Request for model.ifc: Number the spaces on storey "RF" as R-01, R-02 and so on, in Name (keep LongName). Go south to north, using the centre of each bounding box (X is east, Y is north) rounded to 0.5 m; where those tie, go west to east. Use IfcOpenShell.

First a look at what the model holds.

```python
import ifcopenshell
import ifcopenshell.util.element
import ifcopenshell.util.placement

model = ifcopenshell.open("model.ifc")
print(model.schema)
storey = next(s for s in model.by_type("IfcBuildingStorey") if s.Name == "RF")
spaces = [e for e in ifcopenshell.util.element.get_decomposition(storey) if e.is_a("IfcSpace")]
for e in sorted(spaces, key=lambda e: e.id()):
    origin = ifcopenshell.util.placement.get_local_placement(e.ObjectPlacement)[:3, 3]
    print(e.id(), e.Name, e.LongName, origin.round(2) + 0.0, sep=" | ")
```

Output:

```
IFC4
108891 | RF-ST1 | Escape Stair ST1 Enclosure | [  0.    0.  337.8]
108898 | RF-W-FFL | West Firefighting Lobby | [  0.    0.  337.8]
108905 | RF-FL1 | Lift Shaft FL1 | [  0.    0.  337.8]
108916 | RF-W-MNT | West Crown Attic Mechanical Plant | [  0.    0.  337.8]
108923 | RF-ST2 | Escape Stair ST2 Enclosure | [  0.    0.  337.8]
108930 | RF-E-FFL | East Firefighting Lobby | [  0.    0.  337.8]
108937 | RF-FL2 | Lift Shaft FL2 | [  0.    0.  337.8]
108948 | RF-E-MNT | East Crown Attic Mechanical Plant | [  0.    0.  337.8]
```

```python
import ifcopenshell
import ifcopenshell.geom
import ifcopenshell.util.element
import ifcopenshell.util.shape

model = ifcopenshell.open("model.ifc")
settings = ifcopenshell.geom.settings()
settings.set("use-world-coords", True)


def centre(element):
    shape = ifcopenshell.geom.create_shape(settings, element)
    return ifcopenshell.util.shape.get_bbox_centroid(shape.geometry)


storey = next(s for s in model.by_type("IfcBuildingStorey") if s.Name == "RF")
spaces = [e for e in ifcopenshell.util.element.get_decomposition(storey) if e.is_a("IfcSpace")]

# Insertion points can sit at a corner or the storey origin, so sort by the geometry (in metres).
centres = {e: centre(e) for e in spaces}
spaces.sort(key=lambda e: (round(centres[e][1] / 0.5), centres[e][0]))

for i, e in enumerate(spaces, start=1):
    number = f"R-{i:02d}"
    e.Name = number
    print(e.id(), number)

model.write("model_updated.ifc")
```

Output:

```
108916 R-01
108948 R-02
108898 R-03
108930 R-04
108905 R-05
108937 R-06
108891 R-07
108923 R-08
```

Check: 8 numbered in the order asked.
